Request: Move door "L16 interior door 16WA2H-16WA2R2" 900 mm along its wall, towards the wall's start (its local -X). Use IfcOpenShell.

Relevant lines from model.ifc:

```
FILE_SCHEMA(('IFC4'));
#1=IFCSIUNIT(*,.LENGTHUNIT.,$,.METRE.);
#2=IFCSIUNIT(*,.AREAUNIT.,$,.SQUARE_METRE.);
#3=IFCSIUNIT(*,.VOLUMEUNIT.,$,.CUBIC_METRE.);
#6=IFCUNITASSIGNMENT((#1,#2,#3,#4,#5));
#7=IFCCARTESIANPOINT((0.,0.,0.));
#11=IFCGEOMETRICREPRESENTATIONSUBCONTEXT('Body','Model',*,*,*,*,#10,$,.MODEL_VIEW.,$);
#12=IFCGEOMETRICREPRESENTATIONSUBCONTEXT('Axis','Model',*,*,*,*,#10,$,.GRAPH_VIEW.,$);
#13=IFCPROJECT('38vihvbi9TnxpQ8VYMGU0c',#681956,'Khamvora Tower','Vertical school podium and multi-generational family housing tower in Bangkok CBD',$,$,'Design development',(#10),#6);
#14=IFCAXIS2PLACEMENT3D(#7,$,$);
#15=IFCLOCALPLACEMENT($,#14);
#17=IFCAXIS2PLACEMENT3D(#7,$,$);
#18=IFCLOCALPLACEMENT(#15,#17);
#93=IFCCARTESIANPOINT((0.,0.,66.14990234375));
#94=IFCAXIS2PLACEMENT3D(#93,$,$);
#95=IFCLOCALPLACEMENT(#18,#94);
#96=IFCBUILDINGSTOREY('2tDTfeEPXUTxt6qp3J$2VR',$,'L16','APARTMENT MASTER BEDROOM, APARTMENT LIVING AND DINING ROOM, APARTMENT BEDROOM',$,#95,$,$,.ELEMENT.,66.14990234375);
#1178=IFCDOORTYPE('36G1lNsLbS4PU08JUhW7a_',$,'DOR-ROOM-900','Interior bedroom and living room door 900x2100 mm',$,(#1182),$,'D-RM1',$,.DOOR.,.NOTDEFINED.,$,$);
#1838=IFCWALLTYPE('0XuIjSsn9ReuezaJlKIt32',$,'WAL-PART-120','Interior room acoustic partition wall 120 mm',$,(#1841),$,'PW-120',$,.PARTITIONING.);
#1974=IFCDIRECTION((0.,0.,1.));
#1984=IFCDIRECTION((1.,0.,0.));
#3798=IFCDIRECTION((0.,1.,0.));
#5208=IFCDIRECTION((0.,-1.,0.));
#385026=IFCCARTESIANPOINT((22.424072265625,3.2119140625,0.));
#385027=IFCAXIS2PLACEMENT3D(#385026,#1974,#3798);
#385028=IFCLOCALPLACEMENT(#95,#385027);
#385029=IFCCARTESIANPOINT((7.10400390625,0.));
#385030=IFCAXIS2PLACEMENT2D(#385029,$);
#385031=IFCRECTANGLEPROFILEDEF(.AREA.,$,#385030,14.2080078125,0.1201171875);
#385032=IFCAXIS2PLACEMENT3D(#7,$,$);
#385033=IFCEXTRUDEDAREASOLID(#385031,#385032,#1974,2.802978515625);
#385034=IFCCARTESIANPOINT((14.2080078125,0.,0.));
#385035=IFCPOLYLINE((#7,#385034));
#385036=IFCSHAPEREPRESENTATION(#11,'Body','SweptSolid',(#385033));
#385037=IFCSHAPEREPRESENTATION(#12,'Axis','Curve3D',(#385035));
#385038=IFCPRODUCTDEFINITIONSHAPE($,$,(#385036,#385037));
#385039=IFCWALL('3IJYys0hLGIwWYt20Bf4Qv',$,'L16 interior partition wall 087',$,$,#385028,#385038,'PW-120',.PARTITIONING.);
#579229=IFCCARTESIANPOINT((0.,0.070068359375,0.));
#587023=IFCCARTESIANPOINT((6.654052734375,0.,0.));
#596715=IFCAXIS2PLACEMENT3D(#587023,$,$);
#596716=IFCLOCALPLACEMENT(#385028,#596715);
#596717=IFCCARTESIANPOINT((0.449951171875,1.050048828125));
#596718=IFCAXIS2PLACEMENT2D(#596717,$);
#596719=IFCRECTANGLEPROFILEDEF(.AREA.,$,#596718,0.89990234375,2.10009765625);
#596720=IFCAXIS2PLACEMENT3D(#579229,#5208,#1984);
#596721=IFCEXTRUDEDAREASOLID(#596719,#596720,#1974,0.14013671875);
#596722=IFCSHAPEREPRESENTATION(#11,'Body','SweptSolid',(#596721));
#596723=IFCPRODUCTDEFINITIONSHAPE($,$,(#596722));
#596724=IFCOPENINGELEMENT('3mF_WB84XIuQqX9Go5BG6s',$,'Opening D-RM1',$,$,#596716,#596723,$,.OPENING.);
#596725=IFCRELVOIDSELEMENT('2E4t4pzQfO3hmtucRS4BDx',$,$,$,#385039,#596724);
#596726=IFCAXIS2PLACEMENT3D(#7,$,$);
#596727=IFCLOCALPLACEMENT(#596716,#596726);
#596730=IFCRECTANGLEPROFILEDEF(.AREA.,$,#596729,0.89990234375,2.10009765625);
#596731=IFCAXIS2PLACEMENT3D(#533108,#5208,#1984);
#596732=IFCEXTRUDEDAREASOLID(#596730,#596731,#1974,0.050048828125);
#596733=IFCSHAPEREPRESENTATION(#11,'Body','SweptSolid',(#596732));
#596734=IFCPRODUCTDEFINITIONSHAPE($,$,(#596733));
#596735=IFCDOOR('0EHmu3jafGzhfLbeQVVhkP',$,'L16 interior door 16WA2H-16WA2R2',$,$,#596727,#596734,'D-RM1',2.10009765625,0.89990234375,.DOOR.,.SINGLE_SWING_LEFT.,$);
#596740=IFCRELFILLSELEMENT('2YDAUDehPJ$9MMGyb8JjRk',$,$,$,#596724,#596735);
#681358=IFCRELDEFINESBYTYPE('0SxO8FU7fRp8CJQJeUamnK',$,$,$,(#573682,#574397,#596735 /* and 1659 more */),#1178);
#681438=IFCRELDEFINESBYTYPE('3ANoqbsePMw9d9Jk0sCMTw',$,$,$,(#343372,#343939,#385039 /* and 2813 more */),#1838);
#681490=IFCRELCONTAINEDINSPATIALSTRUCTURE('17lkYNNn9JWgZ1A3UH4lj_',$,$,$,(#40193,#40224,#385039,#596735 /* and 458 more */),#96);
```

```python
import ifcopenshell
import ifcopenshell.api.geometry
import ifcopenshell.util.placement

model = ifcopenshell.open("model.ifc")

door = model.by_guid("0EHmu3jafGzhfLbeQVVhkP")
opening = door.FillsVoids[0].RelatingOpeningElement
wall = opening.VoidsElements[0].RelatingBuildingElement

wall_matrix = ifcopenshell.util.placement.get_local_placement(wall.ObjectPlacement)
shift = wall_matrix[:3, 0] * -0.9
before = ifcopenshell.util.placement.get_local_placement(door.ObjectPlacement)[:3, 3].copy()

# The door is placed relative to its opening, so it follows when the opening moves.
matrix = ifcopenshell.util.placement.get_local_placement(opening.ObjectPlacement)
matrix[:3, 3] += shift
ifcopenshell.api.geometry.edit_object_placement(
    model, product=opening, matrix=matrix, is_si=False, should_transform_children=True
)

after = ifcopenshell.util.placement.get_local_placement(door.ObjectPlacement)[:3, 3]
print("door moved by", (after - before).round(3) + 0.0)

model.write("model-out.ifc")
```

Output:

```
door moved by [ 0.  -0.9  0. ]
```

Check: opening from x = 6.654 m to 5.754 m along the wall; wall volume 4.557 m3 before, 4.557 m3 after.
